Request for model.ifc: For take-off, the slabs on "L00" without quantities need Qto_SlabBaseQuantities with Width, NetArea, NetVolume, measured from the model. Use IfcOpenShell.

First a look at what the model holds.

```python
import ifcopenshell
import ifcopenshell.util.element
import ifcopenshell.util.unit

model = ifcopenshell.open("model.ifc")
print(model.schema)
for unit_type in ("LENGTHUNIT", "AREAUNIT", "VOLUMEUNIT"):
    print(unit_type, ifcopenshell.util.unit.calculate_unit_scale(model, unit_type))
storey = next(s for s in model.by_type("IfcBuildingStorey") if s.Name == "L00")
slabs = [e for e in ifcopenshell.util.element.get_decomposition(storey) if e.is_a("IfcSlab")]
for e in sorted(slabs, key=lambda e: e.id()):
    print(e.id(), e.is_a(), e.Name, list(ifcopenshell.util.element.get_psets(e, qtos_only=True)), sep=" | ")
```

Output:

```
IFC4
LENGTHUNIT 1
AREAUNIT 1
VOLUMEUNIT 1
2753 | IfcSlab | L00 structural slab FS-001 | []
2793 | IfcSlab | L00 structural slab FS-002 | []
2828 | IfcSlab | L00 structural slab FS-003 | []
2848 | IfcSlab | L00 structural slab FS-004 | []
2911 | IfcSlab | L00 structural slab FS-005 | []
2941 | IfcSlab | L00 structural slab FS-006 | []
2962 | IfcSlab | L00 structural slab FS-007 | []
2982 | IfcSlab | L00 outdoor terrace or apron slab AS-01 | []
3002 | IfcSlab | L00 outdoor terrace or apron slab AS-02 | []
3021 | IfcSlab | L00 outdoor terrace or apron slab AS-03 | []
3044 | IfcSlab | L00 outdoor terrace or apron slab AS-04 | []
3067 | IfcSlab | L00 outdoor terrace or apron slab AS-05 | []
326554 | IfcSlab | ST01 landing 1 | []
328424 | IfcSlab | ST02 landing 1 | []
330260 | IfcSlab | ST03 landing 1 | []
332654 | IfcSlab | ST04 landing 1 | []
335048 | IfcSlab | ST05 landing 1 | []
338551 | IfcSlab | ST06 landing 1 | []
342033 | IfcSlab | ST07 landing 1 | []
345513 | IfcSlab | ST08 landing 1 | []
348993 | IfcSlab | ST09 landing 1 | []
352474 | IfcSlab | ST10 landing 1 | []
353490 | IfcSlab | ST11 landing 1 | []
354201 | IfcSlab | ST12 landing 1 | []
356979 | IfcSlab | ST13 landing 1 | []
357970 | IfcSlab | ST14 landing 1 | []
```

```python
import ifcopenshell
import ifcopenshell.api.pset
import ifcopenshell.geom
import ifcopenshell.util.element
import ifcopenshell.util.shape
import ifcopenshell.util.unit

model = ifcopenshell.open("model.ifc")
unit_scale = ifcopenshell.util.unit.calculate_unit_scale(model)
area_scale = ifcopenshell.util.unit.calculate_unit_scale(model, "AREAUNIT")
volume_scale = ifcopenshell.util.unit.calculate_unit_scale(model, "VOLUMEUNIT")
settings = ifcopenshell.geom.settings()

storey = next(s for s in model.by_type("IfcBuildingStorey") if s.Name == "L00")
slabs = [e for e in ifcopenshell.util.element.get_decomposition(storey) if e.is_a("IfcSlab")]

for e in sorted(slabs, key=lambda e: e.id()):
    if ifcopenshell.util.element.get_psets(e, qtos_only=True, should_inherit=False):
        continue
    # Geometry comes back in metres, in the element's own axes.
    shape = ifcopenshell.geom.create_shape(settings, e)
    values = {
        "Width": ifcopenshell.util.shape.get_z(shape.geometry) / unit_scale,
        "NetArea": ifcopenshell.util.shape.get_footprint_area(shape.geometry) / area_scale,
        "NetVolume": ifcopenshell.util.shape.get_volume(shape.geometry) / volume_scale,
    }
    qto = ifcopenshell.api.pset.add_qto(model, product=e, name="Qto_SlabBaseQuantities")
    ifcopenshell.api.pset.edit_qto(model, qto=qto, properties=values)
    print(e.id(), {k: round(v, 3) for k, v in values.items()})

model.write("model-out.ifc")
```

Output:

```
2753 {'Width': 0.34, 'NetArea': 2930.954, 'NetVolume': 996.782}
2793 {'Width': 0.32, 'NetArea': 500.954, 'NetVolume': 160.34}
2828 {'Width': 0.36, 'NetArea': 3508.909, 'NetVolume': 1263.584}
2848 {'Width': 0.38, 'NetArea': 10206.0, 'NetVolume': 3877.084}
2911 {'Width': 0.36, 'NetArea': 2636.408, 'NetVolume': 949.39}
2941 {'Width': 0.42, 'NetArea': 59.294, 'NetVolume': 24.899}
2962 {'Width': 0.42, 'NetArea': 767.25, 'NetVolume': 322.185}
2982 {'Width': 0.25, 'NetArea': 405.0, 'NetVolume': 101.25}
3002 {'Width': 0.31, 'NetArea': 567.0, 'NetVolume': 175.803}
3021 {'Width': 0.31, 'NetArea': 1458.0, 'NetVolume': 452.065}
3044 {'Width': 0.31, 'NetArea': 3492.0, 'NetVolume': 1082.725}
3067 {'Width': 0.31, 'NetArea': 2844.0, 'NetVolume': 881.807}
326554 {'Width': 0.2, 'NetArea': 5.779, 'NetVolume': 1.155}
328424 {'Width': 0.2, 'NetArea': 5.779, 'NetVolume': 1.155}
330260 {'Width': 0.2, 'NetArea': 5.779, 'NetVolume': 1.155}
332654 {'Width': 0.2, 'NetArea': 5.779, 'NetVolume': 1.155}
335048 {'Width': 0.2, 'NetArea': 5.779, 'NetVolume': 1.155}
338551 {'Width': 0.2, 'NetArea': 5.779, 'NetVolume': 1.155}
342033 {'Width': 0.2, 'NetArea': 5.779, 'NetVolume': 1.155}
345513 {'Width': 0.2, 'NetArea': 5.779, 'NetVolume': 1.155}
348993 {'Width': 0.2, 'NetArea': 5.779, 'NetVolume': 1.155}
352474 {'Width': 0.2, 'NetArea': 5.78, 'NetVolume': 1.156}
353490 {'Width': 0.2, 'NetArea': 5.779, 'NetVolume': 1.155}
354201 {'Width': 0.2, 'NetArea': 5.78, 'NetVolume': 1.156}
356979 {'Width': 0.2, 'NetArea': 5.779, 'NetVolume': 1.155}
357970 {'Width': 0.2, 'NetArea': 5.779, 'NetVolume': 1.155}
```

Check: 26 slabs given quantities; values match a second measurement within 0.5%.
